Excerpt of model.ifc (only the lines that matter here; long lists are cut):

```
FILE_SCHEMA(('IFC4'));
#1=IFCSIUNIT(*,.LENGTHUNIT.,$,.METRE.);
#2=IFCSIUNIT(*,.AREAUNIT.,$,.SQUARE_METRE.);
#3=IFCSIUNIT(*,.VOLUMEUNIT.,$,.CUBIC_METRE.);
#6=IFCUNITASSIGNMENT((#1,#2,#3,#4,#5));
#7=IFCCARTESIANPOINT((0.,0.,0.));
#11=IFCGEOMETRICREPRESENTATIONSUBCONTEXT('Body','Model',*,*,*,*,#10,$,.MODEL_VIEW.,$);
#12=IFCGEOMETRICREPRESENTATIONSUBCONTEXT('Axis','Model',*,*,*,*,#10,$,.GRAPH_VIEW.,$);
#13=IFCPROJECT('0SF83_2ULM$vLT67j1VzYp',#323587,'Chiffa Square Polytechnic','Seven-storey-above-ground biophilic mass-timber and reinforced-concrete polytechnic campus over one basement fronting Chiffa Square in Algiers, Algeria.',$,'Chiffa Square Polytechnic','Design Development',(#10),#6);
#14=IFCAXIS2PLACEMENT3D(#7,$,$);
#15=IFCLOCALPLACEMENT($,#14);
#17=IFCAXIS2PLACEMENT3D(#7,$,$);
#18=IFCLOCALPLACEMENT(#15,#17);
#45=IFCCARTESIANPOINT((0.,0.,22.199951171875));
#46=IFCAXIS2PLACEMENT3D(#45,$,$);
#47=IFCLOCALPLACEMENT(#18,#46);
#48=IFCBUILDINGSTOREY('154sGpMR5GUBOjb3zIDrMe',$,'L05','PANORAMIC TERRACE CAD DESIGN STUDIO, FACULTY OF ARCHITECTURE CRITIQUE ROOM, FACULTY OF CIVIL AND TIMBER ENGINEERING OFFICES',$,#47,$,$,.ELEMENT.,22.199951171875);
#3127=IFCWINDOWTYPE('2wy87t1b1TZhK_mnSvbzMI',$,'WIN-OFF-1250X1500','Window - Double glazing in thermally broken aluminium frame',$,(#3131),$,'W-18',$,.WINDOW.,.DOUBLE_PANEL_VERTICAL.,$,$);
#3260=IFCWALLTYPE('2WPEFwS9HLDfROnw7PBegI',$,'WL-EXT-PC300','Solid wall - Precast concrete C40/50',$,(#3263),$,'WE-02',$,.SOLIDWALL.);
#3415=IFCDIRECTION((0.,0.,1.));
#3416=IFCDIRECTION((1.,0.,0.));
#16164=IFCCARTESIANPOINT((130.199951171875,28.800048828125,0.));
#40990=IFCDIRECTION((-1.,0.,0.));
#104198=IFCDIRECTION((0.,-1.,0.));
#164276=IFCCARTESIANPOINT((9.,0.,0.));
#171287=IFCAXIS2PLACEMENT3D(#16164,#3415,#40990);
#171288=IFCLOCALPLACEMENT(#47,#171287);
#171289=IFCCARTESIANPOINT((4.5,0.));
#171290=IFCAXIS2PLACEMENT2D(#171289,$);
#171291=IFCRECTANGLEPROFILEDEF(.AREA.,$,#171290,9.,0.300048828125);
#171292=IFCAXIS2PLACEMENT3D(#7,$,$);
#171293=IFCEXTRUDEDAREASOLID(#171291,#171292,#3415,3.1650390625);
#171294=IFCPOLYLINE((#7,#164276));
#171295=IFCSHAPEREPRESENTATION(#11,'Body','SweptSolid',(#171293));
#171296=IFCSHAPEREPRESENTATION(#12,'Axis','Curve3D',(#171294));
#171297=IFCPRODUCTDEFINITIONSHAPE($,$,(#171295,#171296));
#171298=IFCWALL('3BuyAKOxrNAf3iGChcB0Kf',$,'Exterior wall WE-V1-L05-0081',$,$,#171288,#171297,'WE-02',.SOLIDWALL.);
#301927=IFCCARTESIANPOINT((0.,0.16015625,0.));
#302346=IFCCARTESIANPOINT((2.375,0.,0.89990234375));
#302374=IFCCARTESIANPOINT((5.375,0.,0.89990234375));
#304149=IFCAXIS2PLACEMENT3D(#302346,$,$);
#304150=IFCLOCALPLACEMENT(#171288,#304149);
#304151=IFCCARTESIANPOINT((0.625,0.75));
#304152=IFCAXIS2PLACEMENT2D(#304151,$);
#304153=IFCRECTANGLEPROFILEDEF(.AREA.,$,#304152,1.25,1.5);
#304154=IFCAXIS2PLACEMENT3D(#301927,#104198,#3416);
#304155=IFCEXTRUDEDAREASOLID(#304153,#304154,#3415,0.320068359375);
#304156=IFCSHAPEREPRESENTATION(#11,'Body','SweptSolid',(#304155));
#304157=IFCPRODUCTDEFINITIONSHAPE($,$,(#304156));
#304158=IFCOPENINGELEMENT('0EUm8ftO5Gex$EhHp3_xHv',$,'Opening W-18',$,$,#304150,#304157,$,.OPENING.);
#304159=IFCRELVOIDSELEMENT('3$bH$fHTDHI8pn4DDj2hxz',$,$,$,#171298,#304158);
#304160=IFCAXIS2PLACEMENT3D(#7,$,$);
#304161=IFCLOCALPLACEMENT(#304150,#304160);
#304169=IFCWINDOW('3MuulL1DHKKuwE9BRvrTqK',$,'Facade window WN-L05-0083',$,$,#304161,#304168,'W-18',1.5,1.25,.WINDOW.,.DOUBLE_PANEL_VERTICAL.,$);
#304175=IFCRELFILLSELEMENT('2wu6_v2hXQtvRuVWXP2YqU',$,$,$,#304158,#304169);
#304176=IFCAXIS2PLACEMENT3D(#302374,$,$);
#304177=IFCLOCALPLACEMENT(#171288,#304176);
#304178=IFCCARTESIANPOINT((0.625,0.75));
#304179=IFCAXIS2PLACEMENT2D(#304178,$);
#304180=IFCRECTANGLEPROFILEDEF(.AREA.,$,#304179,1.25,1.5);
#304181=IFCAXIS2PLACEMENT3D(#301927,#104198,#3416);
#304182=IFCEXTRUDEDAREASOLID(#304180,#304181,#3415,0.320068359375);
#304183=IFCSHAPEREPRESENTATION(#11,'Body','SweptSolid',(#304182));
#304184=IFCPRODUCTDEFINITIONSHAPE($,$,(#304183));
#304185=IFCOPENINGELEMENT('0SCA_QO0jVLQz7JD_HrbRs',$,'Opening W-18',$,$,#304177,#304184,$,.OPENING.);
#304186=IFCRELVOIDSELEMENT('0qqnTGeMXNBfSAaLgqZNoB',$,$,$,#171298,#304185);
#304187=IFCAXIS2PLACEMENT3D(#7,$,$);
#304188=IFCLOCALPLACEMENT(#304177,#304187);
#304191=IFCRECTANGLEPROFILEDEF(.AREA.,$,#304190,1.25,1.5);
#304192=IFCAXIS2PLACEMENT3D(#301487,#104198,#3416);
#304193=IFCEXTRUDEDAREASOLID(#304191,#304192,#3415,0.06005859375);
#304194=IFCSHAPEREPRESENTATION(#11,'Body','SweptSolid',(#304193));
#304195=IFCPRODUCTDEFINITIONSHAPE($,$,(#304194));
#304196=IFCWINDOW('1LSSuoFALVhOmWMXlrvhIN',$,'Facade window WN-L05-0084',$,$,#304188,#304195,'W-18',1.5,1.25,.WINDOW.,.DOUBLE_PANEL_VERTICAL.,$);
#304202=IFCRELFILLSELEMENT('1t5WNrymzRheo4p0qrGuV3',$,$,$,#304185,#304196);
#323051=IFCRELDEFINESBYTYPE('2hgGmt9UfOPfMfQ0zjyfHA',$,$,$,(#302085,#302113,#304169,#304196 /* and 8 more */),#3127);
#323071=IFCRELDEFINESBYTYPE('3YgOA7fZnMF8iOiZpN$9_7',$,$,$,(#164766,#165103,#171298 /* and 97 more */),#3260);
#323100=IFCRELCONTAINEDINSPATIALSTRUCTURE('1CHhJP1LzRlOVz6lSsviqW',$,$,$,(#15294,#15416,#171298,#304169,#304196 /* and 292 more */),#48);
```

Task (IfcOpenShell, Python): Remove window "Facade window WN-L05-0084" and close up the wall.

```python
import ifcopenshell
import ifcopenshell.api.feature
import ifcopenshell.api.root
import ifcopenshell.geom
import ifcopenshell.util.shape

model = ifcopenshell.open("model.ifc")
settings = ifcopenshell.geom.settings()


def volume(element):
    """Net volume in cubic metres, openings subtracted."""
    shape = ifcopenshell.geom.create_shape(settings, element)
    return ifcopenshell.util.shape.get_volume(shape.geometry)


window = model.by_guid("1LSSuoFALVhOmWMXlrvhIN")
opening = window.FillsVoids[0].RelatingOpeningElement
wall = opening.VoidsElements[0].RelatingBuildingElement
before = volume(wall)

ifcopenshell.api.root.remove_product(model, product=window)
ifcopenshell.api.feature.remove_feature(model, feature=opening)

after = volume(wall)

print(f"wall volume {before:.3f} -> {after:.3f} m3")

model.write("model_updated.ifc")
```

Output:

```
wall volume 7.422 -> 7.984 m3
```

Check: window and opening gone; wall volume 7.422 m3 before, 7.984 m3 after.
